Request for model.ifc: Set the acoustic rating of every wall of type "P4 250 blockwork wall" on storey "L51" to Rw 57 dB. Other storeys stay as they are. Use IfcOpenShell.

First a look at what the model holds.

```python
import ifcopenshell
import ifcopenshell.util.element

model = ifcopenshell.open("model.ifc")
print(model.schema)
storey = next(s for s in model.by_type("IfcBuildingStorey") if s.Name == "L51")
walls = [e for e in ifcopenshell.util.element.get_decomposition(storey) if e.is_a("IfcWall")]
seen = {}
for e in walls:
    element_type = ifcopenshell.util.element.get_type(e)
    key = (element_type.Name if element_type != e and element_type else None, ifcopenshell.util.element.get_pset(e, "Pset_WallCommon", "AcousticRating"))
    seen[key] = seen.get(key, 0) + 1
for (name, value), count in sorted(seen.items(), key=str):
    print(count, "x", name, "|", value)
```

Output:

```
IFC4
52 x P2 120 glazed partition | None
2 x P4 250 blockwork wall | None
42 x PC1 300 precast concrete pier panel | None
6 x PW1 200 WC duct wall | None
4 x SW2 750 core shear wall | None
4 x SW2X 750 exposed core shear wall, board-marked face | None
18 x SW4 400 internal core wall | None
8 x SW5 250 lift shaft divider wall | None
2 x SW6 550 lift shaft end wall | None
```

```python
import ifcopenshell
import ifcopenshell.api.pset
import ifcopenshell.util.element

model = ifcopenshell.open("model.ifc")

storey = next(s for s in model.by_type("IfcBuildingStorey") if s.Name == "L51")
walls = [e for e in ifcopenshell.util.element.get_decomposition(storey) if e.is_a("IfcWall")]

count = 0
for e in walls:
    element_type = ifcopenshell.util.element.get_type(e)
    if element_type in (None, e) or element_type.Name != "P4 250 blockwork wall":
        continue
    # add_pset returns the element's existing set when there is one.
    pset = ifcopenshell.api.pset.add_pset(model, product=e, name="Pset_WallCommon")
    ifcopenshell.api.pset.edit_pset(model, pset=pset, properties={"AcousticRating": "Rw 57 dB"})
    count += 1

print(count, "walls updated")

model.write("model_updated.ifc")
```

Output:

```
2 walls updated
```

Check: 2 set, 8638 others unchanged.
